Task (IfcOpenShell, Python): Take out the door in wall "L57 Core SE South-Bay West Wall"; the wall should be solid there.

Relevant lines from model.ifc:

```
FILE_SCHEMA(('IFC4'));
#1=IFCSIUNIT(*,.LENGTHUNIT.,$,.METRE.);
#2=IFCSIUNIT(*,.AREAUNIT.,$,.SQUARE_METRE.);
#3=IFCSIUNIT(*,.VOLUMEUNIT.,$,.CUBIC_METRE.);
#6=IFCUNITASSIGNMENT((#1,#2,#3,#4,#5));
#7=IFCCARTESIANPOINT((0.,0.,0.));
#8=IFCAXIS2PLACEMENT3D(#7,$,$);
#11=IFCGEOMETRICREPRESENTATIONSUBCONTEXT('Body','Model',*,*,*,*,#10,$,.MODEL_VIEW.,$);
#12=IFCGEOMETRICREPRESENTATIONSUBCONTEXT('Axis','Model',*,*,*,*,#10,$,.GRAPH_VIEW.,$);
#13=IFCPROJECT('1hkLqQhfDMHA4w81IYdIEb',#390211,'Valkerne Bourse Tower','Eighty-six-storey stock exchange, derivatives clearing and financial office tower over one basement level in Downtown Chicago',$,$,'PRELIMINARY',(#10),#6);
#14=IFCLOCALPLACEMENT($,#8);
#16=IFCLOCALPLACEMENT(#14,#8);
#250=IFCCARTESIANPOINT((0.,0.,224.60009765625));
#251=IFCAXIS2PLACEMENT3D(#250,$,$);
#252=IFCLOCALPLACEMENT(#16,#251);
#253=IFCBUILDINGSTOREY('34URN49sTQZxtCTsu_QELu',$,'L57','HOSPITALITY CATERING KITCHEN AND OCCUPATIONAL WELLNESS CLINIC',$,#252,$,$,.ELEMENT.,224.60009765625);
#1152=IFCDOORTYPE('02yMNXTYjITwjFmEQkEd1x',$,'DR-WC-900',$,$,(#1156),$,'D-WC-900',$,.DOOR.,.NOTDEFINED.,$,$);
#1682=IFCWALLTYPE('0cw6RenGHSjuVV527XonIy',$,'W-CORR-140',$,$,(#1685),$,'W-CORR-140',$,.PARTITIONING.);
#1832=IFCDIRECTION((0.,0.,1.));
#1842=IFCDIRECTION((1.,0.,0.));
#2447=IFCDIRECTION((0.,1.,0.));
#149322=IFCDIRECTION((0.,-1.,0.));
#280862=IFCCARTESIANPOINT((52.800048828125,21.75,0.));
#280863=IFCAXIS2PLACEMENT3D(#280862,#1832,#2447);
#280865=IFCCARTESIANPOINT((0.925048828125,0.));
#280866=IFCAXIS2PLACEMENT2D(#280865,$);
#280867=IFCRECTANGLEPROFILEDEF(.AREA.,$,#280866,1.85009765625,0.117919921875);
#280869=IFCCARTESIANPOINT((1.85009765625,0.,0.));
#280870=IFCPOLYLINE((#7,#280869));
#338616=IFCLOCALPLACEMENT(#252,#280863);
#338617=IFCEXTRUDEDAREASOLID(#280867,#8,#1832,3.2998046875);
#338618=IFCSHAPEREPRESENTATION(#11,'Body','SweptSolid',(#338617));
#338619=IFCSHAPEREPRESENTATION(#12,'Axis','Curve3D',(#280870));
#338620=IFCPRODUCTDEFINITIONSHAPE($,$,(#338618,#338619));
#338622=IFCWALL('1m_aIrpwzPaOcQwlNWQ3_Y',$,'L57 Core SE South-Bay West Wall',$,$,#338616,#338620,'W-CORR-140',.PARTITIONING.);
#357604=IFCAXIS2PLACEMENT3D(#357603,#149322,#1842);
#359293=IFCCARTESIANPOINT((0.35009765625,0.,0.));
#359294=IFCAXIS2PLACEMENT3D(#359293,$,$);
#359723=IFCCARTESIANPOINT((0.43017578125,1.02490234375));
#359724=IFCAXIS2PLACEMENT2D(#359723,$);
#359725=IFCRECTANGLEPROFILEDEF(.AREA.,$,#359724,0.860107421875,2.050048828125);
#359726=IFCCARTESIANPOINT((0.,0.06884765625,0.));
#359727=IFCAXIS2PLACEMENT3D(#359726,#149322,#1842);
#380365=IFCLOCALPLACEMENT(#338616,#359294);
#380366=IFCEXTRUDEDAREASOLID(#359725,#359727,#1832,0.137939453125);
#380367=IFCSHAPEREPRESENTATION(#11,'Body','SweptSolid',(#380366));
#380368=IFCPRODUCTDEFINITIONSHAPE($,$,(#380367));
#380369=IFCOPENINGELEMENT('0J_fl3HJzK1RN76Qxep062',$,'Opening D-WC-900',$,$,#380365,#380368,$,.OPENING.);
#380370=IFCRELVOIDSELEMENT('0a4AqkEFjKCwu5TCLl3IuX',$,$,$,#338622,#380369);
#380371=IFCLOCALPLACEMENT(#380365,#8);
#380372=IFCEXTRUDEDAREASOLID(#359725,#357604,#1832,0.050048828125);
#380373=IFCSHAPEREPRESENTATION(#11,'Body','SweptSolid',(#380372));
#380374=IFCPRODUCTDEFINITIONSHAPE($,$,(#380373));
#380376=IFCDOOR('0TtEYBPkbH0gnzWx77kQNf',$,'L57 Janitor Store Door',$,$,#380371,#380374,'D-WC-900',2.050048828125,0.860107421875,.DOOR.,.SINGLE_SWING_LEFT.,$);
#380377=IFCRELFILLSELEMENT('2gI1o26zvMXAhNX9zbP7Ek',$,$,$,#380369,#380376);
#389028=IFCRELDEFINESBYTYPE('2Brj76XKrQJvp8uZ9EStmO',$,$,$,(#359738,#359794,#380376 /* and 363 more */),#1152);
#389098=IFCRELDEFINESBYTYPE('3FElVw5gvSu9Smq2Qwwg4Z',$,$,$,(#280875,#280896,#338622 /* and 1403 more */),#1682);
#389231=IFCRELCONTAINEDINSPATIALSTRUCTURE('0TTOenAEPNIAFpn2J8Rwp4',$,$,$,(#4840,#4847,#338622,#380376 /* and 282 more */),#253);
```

```python
import ifcopenshell
import ifcopenshell.api.feature
import ifcopenshell.api.root
import ifcopenshell.geom
import ifcopenshell.util.shape

model = ifcopenshell.open("model.ifc")
settings = ifcopenshell.geom.settings()


def volume(element):
    """Net volume in cubic metres, openings subtracted."""
    shape = ifcopenshell.geom.create_shape(settings, element)
    return ifcopenshell.util.shape.get_volume(shape.geometry)


door = model.by_guid("0TtEYBPkbH0gnzWx77kQNf")
opening = door.FillsVoids[0].RelatingOpeningElement
wall = opening.VoidsElements[0].RelatingBuildingElement
before = volume(wall)

ifcopenshell.api.root.remove_product(model, product=door)
ifcopenshell.api.feature.remove_feature(model, feature=opening)

after = volume(wall)

print(f"wall volume {before:.3f} -> {after:.3f} m3")

model.write("model_edited.ifc")
```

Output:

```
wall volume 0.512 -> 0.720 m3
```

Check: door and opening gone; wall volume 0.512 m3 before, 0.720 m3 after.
